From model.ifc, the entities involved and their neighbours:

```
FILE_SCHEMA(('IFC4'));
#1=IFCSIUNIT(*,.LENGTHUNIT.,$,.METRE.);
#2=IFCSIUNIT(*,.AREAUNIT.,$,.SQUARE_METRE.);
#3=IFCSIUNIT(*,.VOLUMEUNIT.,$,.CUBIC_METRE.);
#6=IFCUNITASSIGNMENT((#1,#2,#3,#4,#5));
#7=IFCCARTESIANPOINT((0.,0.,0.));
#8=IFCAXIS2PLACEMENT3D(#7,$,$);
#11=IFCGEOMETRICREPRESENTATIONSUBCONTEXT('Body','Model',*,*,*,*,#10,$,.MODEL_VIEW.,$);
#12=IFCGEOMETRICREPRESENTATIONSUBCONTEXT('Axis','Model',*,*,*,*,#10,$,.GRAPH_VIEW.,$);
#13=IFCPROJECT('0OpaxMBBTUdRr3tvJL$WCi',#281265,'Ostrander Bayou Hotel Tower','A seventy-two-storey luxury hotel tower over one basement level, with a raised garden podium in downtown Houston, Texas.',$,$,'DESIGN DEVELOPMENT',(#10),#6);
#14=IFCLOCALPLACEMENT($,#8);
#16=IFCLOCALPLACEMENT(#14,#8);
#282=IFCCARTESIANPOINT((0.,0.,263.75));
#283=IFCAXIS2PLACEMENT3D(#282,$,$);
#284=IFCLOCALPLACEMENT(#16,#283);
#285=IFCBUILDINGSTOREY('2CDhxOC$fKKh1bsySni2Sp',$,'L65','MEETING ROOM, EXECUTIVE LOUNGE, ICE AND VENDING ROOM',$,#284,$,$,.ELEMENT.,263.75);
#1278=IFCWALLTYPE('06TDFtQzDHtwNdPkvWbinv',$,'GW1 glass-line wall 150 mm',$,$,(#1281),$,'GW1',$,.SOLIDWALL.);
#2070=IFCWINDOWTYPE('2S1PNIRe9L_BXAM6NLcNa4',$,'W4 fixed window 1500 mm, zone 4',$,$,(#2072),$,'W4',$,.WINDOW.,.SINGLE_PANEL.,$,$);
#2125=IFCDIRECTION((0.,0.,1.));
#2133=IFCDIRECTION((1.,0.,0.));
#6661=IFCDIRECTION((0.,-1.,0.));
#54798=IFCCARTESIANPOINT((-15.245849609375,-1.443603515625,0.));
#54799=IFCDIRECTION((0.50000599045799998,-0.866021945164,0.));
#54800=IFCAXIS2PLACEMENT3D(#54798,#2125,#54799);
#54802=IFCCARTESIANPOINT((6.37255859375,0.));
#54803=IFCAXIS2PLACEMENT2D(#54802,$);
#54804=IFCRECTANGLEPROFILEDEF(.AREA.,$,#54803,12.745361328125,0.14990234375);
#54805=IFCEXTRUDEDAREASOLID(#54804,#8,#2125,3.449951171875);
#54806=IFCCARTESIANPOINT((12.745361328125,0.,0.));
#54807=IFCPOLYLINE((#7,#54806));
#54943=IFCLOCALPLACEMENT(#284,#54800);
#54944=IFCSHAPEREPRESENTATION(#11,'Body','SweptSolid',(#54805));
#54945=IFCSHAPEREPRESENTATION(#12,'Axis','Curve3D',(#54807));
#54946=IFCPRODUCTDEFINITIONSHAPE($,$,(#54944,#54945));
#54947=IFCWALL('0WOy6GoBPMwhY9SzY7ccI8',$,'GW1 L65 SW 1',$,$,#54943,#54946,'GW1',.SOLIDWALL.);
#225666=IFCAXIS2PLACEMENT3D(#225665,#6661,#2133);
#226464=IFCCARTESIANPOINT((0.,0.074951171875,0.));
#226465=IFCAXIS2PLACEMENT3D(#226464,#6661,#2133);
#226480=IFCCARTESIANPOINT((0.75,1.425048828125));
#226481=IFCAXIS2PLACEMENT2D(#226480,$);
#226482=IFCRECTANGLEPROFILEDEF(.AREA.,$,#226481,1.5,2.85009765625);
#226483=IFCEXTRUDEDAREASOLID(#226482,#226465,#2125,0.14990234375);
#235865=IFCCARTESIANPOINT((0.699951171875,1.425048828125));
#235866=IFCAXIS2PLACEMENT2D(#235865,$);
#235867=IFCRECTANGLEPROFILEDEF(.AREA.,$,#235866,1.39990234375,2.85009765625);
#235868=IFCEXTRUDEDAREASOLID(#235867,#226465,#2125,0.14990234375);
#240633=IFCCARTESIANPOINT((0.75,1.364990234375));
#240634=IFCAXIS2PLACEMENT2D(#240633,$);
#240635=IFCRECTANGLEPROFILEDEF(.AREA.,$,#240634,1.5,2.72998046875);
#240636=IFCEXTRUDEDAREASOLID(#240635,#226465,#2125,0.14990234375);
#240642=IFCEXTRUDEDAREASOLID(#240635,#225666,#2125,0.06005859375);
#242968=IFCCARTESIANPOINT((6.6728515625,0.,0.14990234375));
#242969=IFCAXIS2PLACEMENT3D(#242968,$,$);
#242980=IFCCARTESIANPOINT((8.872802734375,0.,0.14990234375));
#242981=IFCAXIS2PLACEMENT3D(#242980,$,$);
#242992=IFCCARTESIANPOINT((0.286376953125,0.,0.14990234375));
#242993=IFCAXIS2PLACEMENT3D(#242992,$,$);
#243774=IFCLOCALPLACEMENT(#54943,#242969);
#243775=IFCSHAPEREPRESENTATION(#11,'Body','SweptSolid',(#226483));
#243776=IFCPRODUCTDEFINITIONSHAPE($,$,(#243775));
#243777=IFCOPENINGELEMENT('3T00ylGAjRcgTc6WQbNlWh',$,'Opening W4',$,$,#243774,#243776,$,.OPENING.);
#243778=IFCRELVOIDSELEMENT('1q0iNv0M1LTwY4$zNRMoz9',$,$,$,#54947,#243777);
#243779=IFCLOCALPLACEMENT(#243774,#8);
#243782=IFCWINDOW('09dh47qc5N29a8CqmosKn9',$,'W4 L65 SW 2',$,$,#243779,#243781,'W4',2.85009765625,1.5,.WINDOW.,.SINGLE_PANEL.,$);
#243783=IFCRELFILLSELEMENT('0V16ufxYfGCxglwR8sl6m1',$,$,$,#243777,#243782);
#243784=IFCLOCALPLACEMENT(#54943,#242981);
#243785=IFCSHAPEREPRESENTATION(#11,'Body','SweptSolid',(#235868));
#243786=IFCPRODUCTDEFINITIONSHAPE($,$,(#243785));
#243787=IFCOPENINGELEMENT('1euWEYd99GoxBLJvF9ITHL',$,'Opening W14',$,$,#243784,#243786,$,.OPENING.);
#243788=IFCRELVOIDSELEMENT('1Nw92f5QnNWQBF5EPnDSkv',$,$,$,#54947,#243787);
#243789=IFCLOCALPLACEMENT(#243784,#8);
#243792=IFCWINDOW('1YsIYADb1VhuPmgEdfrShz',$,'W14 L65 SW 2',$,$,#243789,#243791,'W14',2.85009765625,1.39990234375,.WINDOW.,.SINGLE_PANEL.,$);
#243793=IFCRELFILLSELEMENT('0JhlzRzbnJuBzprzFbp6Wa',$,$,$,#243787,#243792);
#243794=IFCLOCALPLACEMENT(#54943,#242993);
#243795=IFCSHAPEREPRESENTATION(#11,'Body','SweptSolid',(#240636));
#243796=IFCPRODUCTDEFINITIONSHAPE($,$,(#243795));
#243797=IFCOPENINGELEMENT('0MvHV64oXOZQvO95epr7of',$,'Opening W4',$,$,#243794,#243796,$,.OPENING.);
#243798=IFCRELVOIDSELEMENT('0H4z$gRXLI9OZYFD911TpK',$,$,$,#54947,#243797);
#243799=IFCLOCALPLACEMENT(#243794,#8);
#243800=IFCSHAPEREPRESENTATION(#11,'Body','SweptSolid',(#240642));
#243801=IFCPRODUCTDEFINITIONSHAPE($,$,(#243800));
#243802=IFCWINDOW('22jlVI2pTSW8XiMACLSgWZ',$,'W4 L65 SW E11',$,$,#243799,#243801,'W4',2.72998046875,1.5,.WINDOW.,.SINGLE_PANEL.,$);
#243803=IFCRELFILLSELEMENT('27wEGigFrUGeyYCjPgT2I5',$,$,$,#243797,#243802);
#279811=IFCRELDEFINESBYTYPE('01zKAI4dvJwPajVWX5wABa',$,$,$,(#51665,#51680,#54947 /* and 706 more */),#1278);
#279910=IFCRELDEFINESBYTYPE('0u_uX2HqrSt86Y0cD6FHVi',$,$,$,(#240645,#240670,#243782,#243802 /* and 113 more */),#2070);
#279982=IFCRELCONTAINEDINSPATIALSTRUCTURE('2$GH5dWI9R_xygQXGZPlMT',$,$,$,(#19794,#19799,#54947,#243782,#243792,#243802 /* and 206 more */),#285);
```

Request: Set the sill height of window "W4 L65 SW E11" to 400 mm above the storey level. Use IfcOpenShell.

```python
import numpy as np
import ifcopenshell
import ifcopenshell.api.geometry
import ifcopenshell.geom
import ifcopenshell.util.element
import ifcopenshell.util.placement
import ifcopenshell.util.shape
import ifcopenshell.util.unit

model = ifcopenshell.open("model.ifc")
unit_scale = ifcopenshell.util.unit.calculate_unit_scale(model)

window = model.by_guid("22jlVI2pTSW8XiMACLSgWZ")
opening = window.FillsVoids[0].RelatingOpeningElement
storey = ifcopenshell.util.element.get_container(window, ifc_class="IfcBuildingStorey")
level = ifcopenshell.util.placement.get_local_placement(storey.ObjectPlacement)[2, 3]

# The opening's origin need not be at the sill, so measure its lowest point.
shape = ifcopenshell.geom.create_shape(ifcopenshell.geom.settings(), opening)
bottom = ifcopenshell.util.shape.get_shape_bottom_elevation(shape, shape.geometry) / unit_scale
dz = level + 0.4 / unit_scale - bottom

shift = np.array([0.0, 0.0, dz])
# The window is placed relative to its opening, so it follows when the opening moves.
matrix = ifcopenshell.util.placement.get_local_placement(opening.ObjectPlacement)
matrix[:3, 3] += shift
ifcopenshell.api.geometry.edit_object_placement(
    model, product=opening, matrix=matrix, is_si=False, should_transform_children=True
)

print(f"moved by {dz * unit_scale:+.3f} m")

model.write("model_updated.ifc")
```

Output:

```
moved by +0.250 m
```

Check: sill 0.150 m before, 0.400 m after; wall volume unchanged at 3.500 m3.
